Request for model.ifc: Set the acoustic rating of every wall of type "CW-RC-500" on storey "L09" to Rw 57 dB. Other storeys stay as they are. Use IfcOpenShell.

First a look at what the model holds.

```python
import ifcopenshell
import ifcopenshell.util.element

model = ifcopenshell.open("model.ifc")
print(model.schema)
storey = next(s for s in model.by_type("IfcBuildingStorey") if s.Name == "L09")
walls = [e for e in ifcopenshell.util.element.get_decomposition(storey) if e.is_a("IfcWall")]
seen = {}
for e in walls:
    element_type = ifcopenshell.util.element.get_type(e)
    key = (element_type.Name if element_type != e and element_type else None, ifcopenshell.util.element.get_pset(e, "Pset_WallCommon", "AcousticRating"))
    seen[key] = seen.get(key, 0) + 1
for (name, value), count in sorted(seen.items(), key=str):
    print(count, "x", name, "|", value)
```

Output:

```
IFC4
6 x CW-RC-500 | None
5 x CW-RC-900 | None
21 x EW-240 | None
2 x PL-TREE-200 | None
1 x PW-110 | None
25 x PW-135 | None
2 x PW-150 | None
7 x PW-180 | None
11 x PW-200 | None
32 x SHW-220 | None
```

```python
import ifcopenshell
import ifcopenshell.api.pset
import ifcopenshell.util.element

model = ifcopenshell.open("model.ifc")

storey = next(s for s in model.by_type("IfcBuildingStorey") if s.Name == "L09")
walls = [e for e in ifcopenshell.util.element.get_decomposition(storey) if e.is_a("IfcWall")]

count = 0
for e in walls:
    element_type = ifcopenshell.util.element.get_type(e)
    if element_type in (None, e) or element_type.Name != "CW-RC-500":
        continue
    found = ifcopenshell.util.element.get_pset(e, "Pset_WallCommon", should_inherit=False)
    if found:
        pset = model.by_id(found["id"])
        if len(ifcopenshell.util.element.get_elements_by_pset(pset)) > 1:
            pset = ifcopenshell.api.pset.unshare_pset(model, products=[e], pset=pset)[0]
    else:
        pset = ifcopenshell.api.pset.add_pset(model, product=e, name="Pset_WallCommon")
    ifcopenshell.api.pset.edit_pset(model, pset=pset, properties={"AcousticRating": "Rw 57 dB"})
    count += 1

print(count, "walls updated")

model.write("model_rev.ifc")
```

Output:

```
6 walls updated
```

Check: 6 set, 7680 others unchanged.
